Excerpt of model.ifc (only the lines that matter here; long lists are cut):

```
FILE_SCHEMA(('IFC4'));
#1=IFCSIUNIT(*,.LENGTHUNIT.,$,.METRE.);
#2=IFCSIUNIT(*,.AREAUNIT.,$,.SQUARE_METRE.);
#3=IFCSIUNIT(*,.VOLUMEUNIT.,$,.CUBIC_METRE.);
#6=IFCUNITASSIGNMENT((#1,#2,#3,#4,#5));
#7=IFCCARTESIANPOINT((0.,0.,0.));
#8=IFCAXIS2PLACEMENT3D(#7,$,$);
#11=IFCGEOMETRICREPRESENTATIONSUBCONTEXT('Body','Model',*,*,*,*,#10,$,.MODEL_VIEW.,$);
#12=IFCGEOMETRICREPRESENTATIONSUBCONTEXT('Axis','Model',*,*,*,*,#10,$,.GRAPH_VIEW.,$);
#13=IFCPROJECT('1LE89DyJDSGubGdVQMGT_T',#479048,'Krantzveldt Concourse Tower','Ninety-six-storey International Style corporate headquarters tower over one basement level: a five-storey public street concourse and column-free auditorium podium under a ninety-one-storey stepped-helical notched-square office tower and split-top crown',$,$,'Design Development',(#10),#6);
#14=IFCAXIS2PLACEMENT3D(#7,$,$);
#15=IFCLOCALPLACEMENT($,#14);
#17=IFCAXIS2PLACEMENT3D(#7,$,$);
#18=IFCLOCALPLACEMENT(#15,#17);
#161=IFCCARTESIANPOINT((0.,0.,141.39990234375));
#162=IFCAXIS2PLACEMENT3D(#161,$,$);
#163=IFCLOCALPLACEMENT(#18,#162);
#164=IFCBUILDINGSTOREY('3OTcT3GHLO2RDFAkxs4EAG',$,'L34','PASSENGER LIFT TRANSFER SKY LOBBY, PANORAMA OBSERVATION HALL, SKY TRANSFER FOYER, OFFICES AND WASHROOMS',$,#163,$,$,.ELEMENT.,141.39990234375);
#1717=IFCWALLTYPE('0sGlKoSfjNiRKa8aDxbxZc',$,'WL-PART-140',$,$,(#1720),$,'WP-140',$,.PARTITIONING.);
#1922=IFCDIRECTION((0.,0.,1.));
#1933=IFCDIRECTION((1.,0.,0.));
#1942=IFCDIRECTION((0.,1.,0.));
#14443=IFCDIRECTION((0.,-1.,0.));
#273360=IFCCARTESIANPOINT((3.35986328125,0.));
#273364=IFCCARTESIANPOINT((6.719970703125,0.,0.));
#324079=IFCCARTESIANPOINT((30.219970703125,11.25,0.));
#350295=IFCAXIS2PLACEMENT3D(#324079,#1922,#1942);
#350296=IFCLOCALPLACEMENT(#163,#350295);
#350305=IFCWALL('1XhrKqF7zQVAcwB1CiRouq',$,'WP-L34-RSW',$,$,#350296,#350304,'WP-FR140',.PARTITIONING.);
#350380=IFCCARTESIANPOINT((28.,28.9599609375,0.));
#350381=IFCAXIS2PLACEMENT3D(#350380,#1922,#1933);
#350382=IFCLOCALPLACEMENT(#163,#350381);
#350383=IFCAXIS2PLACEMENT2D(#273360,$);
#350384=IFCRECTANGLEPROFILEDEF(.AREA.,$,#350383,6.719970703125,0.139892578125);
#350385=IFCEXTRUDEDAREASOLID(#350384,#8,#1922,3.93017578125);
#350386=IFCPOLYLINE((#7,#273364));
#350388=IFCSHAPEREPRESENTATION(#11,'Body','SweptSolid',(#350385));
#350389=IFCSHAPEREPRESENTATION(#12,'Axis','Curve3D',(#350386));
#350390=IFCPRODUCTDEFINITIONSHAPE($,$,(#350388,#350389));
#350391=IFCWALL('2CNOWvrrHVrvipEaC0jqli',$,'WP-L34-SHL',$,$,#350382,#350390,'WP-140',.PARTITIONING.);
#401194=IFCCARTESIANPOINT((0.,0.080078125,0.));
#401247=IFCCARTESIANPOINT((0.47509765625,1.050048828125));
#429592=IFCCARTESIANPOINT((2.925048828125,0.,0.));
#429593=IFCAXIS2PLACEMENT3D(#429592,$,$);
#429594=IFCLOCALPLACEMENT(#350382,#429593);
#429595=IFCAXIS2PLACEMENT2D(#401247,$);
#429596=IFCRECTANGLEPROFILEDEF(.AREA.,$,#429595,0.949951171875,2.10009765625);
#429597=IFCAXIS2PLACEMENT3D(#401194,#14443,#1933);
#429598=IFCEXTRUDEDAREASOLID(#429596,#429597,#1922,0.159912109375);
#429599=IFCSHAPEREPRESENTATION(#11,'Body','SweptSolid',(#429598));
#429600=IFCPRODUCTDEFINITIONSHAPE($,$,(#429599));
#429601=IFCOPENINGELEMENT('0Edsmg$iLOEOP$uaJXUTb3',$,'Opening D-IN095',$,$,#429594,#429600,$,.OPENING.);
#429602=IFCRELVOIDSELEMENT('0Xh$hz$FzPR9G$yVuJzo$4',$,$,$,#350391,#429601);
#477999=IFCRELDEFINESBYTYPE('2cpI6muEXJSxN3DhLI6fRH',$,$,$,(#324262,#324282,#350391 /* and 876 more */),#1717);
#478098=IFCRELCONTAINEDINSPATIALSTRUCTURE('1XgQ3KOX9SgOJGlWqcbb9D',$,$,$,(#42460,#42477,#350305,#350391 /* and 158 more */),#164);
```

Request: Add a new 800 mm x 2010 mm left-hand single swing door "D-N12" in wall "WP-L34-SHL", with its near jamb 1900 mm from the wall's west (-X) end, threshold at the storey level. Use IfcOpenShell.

```python
import numpy as np
import ifcopenshell
import ifcopenshell.api.feature
import ifcopenshell.api.geometry
import ifcopenshell.api.root
import ifcopenshell.api.spatial
import ifcopenshell.geom
import ifcopenshell.util.element
import ifcopenshell.util.placement
import ifcopenshell.util.representation
import ifcopenshell.util.shape
import ifcopenshell.util.unit

model = ifcopenshell.open("model.ifc")
unit_scale = ifcopenshell.util.unit.calculate_unit_scale(model)
settings = ifcopenshell.geom.settings()


def volume(element):
    """Net volume in cubic metres, openings subtracted."""
    shape = ifcopenshell.geom.create_shape(settings, element)
    return ifcopenshell.util.shape.get_volume(shape.geometry)


wall = model.by_id(350391)
storey = ifcopenshell.util.element.get_container(wall, ifc_class="IfcBuildingStorey")
context = ifcopenshell.util.representation.get_context(model, "Model", "Body", "MODEL_VIEW")
before = volume(wall)

width, height, from_end, sill = 0.8, 2.01, 1.9, 0.0  # metres

# The wall runs along its own X axis, and the end named is its -X end.
wall_shape = ifcopenshell.geom.create_shape(settings, wall)
x, y, z = ifcopenshell.util.shape.get_vertices(wall_shape.geometry).T
start = x.min() + from_end
face, thickness = float(y.min()), float(y.max() - y.min())
wall_matrix = ifcopenshell.util.placement.get_local_placement(wall.ObjectPlacement)
level = ifcopenshell.util.placement.get_local_placement(storey.ObjectPlacement)[2, 3]


def in_wall(x, y):
    """Placement at x, y metres in the wall's axes, at sill height."""
    matrix = wall_matrix.copy()
    matrix[:, 3] = wall_matrix @ np.array([x / unit_scale, y / unit_scale, 0.0, 1.0])
    matrix[2, 3] = level + sill / unit_scale
    return matrix


# Opening: a box that overshoots both wall faces by 50 mm.
opening = ifcopenshell.api.root.create_entity(model, ifc_class="IfcOpeningElement", predefined_type="OPENING")
box = ifcopenshell.api.geometry.add_wall_representation(
    model, context=context, length=width, height=height, thickness=thickness + 0.1
)
ifcopenshell.api.geometry.assign_representation(model, product=opening, representation=box)
ifcopenshell.api.geometry.edit_object_placement(model, product=opening, matrix=in_wall(start, face - 0.05), is_si=False)
ifcopenshell.api.feature.add_feature(model, feature=opening, element=wall)

door = ifcopenshell.api.root.create_entity(model, ifc_class="IfcDoor", name="D-N12", predefined_type="DOOR")
door.OverallWidth, door.OverallHeight = width / unit_scale, height / unit_scale
door.OperationType = "SINGLE_SWING_LEFT"
body = ifcopenshell.api.geometry.add_door_representation(
    model,
    context=context,
    overall_width=door.OverallWidth,
    overall_height=door.OverallHeight,
    operation_type="SINGLE_SWING_LEFT",
    lining_properties={"LiningDepth": thickness / unit_scale, "ThresholdDepth": thickness / unit_scale},
)
ifcopenshell.api.geometry.assign_representation(model, product=door, representation=body)
ifcopenshell.api.spatial.assign_container(model, products=[door], relating_structure=storey)
ifcopenshell.api.feature.add_filling(model, opening=opening, element=door)

# The lining spans the wall, so the door starts at the wall face.
ifcopenshell.api.geometry.edit_object_placement(model, product=door, matrix=in_wall(start, face), is_si=False)

after = volume(wall)

print(f"wall volume {before:.3f} -> {after:.3f} m3")

model.write("model_v2.ifc")
```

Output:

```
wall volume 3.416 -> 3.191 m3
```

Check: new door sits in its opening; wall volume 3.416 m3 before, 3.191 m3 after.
